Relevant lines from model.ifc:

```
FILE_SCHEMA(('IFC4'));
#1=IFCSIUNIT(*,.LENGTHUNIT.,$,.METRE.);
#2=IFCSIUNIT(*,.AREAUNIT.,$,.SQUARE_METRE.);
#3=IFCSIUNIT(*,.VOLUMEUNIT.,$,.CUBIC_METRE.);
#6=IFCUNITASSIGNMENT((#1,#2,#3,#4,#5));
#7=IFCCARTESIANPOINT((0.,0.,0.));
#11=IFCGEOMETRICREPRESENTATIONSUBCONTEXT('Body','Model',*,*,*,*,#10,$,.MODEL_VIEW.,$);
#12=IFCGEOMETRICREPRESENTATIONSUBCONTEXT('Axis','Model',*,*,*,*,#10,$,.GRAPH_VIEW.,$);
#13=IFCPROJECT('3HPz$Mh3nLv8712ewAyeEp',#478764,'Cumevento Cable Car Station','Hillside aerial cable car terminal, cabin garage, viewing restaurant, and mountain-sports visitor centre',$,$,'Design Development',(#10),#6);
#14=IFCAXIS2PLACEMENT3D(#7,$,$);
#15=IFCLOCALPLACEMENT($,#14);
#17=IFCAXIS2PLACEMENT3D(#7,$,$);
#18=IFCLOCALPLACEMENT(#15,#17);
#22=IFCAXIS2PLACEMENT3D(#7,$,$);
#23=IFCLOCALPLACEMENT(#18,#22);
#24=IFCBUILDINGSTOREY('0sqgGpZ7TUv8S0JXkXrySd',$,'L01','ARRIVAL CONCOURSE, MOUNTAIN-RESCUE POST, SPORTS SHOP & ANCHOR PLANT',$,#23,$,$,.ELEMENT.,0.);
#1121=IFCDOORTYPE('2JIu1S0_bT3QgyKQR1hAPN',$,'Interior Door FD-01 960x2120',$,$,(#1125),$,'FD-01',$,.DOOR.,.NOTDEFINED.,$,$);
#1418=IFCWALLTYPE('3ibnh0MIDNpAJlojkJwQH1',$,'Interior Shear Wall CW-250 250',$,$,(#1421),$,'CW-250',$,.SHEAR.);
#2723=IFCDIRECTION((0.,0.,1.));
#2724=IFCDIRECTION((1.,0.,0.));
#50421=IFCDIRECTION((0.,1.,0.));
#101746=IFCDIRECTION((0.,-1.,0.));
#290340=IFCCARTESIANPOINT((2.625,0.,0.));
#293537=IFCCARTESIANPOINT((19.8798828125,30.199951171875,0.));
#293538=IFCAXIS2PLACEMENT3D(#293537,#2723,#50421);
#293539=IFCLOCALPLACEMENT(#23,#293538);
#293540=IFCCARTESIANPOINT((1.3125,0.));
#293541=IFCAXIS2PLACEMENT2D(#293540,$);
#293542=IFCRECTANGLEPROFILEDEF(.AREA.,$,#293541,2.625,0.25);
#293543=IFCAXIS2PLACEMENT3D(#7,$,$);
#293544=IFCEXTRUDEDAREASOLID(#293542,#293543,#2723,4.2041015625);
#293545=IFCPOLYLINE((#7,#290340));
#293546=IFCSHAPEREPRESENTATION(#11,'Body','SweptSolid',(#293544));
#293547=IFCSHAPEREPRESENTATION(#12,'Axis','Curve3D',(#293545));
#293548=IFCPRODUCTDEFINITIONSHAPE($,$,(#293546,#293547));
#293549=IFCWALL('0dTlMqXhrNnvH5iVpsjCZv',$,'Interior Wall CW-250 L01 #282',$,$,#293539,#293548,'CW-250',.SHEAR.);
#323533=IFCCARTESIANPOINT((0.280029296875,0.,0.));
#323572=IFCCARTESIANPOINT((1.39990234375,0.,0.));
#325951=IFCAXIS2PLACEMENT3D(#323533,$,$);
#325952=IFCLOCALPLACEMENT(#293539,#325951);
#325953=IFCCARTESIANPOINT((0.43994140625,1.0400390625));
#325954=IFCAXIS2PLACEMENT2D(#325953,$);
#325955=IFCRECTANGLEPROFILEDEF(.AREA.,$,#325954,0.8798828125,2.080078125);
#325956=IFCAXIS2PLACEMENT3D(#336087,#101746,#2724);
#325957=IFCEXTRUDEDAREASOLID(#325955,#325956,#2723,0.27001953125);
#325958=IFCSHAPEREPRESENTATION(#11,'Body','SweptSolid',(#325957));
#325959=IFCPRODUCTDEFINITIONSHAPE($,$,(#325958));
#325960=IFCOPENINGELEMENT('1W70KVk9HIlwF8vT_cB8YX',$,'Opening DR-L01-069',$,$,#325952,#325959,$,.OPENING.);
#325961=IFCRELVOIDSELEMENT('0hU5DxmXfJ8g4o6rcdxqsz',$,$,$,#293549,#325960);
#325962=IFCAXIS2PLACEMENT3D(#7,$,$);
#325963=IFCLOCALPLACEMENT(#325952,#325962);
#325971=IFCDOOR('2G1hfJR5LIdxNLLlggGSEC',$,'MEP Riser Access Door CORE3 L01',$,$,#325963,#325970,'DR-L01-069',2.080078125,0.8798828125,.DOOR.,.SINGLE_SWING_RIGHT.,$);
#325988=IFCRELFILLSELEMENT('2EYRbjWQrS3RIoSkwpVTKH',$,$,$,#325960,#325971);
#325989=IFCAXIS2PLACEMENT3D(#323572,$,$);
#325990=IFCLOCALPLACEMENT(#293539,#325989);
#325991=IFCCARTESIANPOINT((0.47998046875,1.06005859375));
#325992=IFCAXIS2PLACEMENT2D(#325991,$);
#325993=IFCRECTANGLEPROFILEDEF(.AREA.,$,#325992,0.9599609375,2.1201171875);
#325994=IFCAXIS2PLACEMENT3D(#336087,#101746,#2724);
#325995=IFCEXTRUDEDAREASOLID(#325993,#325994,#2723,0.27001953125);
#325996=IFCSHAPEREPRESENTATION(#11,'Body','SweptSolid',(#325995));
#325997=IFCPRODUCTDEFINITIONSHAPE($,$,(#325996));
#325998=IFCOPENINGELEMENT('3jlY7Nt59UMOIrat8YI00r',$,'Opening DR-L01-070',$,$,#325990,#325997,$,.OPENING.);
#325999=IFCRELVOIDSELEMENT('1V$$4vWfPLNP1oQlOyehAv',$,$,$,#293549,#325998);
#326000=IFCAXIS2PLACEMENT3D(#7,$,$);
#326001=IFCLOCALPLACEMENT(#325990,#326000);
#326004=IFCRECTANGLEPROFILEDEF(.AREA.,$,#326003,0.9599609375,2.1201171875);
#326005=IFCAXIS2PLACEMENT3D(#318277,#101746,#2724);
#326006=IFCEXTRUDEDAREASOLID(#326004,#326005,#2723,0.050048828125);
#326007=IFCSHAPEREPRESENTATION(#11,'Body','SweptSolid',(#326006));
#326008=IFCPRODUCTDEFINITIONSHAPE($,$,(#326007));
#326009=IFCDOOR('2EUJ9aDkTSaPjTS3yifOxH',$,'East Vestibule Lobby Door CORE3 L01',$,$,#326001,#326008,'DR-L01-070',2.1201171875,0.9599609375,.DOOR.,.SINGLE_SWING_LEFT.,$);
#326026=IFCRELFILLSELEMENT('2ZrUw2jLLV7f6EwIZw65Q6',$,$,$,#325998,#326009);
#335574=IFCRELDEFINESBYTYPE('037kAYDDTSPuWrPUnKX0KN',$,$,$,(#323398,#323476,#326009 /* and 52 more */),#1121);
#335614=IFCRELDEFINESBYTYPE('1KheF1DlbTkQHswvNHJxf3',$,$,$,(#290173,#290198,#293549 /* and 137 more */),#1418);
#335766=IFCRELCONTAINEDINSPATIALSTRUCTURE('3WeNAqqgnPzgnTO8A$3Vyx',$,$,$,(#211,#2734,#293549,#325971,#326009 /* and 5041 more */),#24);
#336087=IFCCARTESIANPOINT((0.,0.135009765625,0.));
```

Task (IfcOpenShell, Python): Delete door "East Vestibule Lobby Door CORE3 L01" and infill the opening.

```python
import ifcopenshell
import ifcopenshell.api.feature
import ifcopenshell.api.root
import ifcopenshell.geom
import ifcopenshell.util.shape

model = ifcopenshell.open("model.ifc")
settings = ifcopenshell.geom.settings()


def volume(element):
    """Net volume in cubic metres, openings subtracted."""
    shape = ifcopenshell.geom.create_shape(settings, element)
    return ifcopenshell.util.shape.get_volume(shape.geometry)


door = model.by_id(326009)
opening = door.FillsVoids[0].RelatingOpeningElement
wall = opening.VoidsElements[0].RelatingBuildingElement
before = volume(wall)

ifcopenshell.api.root.remove_product(model, product=door)
ifcopenshell.api.feature.remove_feature(model, feature=opening)

after = volume(wall)

print(f"wall volume {before:.3f} -> {after:.3f} m3")

model.write("model_rev.ifc")
```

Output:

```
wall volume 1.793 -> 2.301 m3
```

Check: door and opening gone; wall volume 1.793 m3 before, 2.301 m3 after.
